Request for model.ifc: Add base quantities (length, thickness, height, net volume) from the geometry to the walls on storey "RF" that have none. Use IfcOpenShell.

First a look at what the model holds.

```python
import ifcopenshell
import ifcopenshell.util.element
import ifcopenshell.util.unit

model = ifcopenshell.open("model.ifc")
print(model.schema)
for unit_type in ("LENGTHUNIT", "AREAUNIT", "VOLUMEUNIT"):
    print(unit_type, ifcopenshell.util.unit.calculate_unit_scale(model, unit_type))
storey = next(s for s in model.by_type("IfcBuildingStorey") if s.Name == "RF")
walls = [e for e in ifcopenshell.util.element.get_decomposition(storey) if e.is_a("IfcWall")]
for e in sorted(walls, key=lambda e: e.id()):
    print(e.id(), e.is_a(), e.Name, list(ifcopenshell.util.element.get_psets(e, qtos_only=True)), sep=" | ")
```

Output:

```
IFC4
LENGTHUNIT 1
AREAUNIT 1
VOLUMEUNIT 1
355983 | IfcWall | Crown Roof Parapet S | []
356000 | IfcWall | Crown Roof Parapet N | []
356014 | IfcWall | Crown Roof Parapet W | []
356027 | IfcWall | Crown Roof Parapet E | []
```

```python
import ifcopenshell
import ifcopenshell.api.pset
import ifcopenshell.geom
import ifcopenshell.util.element
import ifcopenshell.util.shape
import ifcopenshell.util.unit

model = ifcopenshell.open("model.ifc")
unit_scale = ifcopenshell.util.unit.calculate_unit_scale(model)
volume_scale = ifcopenshell.util.unit.calculate_unit_scale(model, "VOLUMEUNIT")
settings = ifcopenshell.geom.settings()

storey = next(s for s in model.by_type("IfcBuildingStorey") if s.Name == "RF")
walls = [e for e in ifcopenshell.util.element.get_decomposition(storey) if e.is_a("IfcWall")]

for e in sorted(walls, key=lambda e: e.id()):
    if ifcopenshell.util.element.get_psets(e, qtos_only=True, should_inherit=False):
        continue
    # Geometry comes back in metres, in the element's own axes.
    shape = ifcopenshell.geom.create_shape(settings, e)
    values = {
        "Length": ifcopenshell.util.shape.get_x(shape.geometry) / unit_scale,
        "Width": ifcopenshell.util.shape.get_y(shape.geometry) / unit_scale,
        "Height": ifcopenshell.util.shape.get_z(shape.geometry) / unit_scale,
        "NetVolume": ifcopenshell.util.shape.get_volume(shape.geometry) / volume_scale,
    }
    qto = ifcopenshell.api.pset.add_qto(model, product=e, name="Qto_WallBaseQuantities")
    ifcopenshell.api.pset.edit_qto(model, qto=qto, properties=values)
    print(e.id(), {k: round(v, 3) for k, v in values.items()})

model.write("model_edited.ifc")
```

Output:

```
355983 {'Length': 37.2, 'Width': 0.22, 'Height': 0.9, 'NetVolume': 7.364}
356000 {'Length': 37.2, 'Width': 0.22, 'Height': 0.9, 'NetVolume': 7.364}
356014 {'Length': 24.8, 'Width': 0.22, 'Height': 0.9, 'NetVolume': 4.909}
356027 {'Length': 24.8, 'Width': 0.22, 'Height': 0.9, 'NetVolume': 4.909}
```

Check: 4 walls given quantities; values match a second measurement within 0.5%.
